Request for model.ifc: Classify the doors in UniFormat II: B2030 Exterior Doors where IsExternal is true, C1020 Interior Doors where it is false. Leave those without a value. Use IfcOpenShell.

First a look at what the model holds.

```python
import ifcopenshell
import ifcopenshell.util.element

model = ifcopenshell.open("model.ifc")
print(model.schema)
print("classifications:", [c.Name for c in model.by_type("IfcClassification")])
values = [ifcopenshell.util.element.get_pset(e, "Pset_DoorCommon", "IsExternal") for e in model.by_type("IfcDoor")]
for value in (True, False, None):
    print("IsExternal", value, values.count(value))
```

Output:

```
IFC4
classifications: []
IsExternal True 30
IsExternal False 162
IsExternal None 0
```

```python
import ifcopenshell
import ifcopenshell.api.classification
import ifcopenshell.util.element

model = ifcopenshell.open("model.ifc")

system = ifcopenshell.api.classification.add_classification(model, classification="UniFormat II")

doors = model.by_type("IfcDoor")
external = {e: ifcopenshell.util.element.get_pset(e, "Pset_DoorCommon", "IsExternal") for e in doors}
for flag, code, name in ((True, "B2030", "Exterior Doors"), (False, "C1020", "Interior Doors")):
    products = [e for e in doors if external[e] is flag]
    ifcopenshell.api.classification.add_reference(
        model, products=products, classification=system, identification=code, name=name
    )
    print(code, len(products))

model.write("model_edited.ifc")
```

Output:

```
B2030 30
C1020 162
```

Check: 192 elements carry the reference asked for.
